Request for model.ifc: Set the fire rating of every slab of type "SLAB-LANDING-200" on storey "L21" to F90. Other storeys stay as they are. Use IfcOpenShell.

First a look at what the model holds.

```python
import ifcopenshell
import ifcopenshell.util.element

model = ifcopenshell.open("model.ifc")
print(model.schema)
storey = next(s for s in model.by_type("IfcBuildingStorey") if s.Name == "L21")
slabs = [e for e in ifcopenshell.util.element.get_decomposition(storey) if e.is_a("IfcSlab")]
seen = {}
for e in slabs:
    element_type = ifcopenshell.util.element.get_type(e)
    key = (element_type.Name if element_type != e and element_type else None, ifcopenshell.util.element.get_pset(e, "Pset_SlabCommon", "FireRating"))
    seen[key] = seen.get(key, 0) + 1
for (name, value), count in sorted(seen.items(), key=str):
    print(count, "x", name, "|", value)
```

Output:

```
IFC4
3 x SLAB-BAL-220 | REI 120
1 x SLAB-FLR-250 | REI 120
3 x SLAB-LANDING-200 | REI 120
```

```python
import ifcopenshell
import ifcopenshell.api.pset
import ifcopenshell.util.element

model = ifcopenshell.open("model.ifc")

storey = next(s for s in model.by_type("IfcBuildingStorey") if s.Name == "L21")
slabs = [e for e in ifcopenshell.util.element.get_decomposition(storey) if e.is_a("IfcSlab")]

count = 0
for e in slabs:
    element_type = ifcopenshell.util.element.get_type(e)
    if element_type in (None, e) or element_type.Name != "SLAB-LANDING-200":
        continue
    found = ifcopenshell.util.element.get_pset(e, "Pset_SlabCommon", should_inherit=False)
    if found:
        pset = model.by_id(found["id"])
        if len(ifcopenshell.util.element.get_elements_by_pset(pset)) > 1:
            pset = ifcopenshell.api.pset.unshare_pset(model, products=[e], pset=pset)[0]
    else:
        pset = ifcopenshell.api.pset.add_pset(model, product=e, name="Pset_SlabCommon")
    ifcopenshell.api.pset.edit_pset(model, pset=pset, properties={"FireRating": "F90"})
    count += 1

print(count, "slabs updated")

model.write("model_v2.ifc")
```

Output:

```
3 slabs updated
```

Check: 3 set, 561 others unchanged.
